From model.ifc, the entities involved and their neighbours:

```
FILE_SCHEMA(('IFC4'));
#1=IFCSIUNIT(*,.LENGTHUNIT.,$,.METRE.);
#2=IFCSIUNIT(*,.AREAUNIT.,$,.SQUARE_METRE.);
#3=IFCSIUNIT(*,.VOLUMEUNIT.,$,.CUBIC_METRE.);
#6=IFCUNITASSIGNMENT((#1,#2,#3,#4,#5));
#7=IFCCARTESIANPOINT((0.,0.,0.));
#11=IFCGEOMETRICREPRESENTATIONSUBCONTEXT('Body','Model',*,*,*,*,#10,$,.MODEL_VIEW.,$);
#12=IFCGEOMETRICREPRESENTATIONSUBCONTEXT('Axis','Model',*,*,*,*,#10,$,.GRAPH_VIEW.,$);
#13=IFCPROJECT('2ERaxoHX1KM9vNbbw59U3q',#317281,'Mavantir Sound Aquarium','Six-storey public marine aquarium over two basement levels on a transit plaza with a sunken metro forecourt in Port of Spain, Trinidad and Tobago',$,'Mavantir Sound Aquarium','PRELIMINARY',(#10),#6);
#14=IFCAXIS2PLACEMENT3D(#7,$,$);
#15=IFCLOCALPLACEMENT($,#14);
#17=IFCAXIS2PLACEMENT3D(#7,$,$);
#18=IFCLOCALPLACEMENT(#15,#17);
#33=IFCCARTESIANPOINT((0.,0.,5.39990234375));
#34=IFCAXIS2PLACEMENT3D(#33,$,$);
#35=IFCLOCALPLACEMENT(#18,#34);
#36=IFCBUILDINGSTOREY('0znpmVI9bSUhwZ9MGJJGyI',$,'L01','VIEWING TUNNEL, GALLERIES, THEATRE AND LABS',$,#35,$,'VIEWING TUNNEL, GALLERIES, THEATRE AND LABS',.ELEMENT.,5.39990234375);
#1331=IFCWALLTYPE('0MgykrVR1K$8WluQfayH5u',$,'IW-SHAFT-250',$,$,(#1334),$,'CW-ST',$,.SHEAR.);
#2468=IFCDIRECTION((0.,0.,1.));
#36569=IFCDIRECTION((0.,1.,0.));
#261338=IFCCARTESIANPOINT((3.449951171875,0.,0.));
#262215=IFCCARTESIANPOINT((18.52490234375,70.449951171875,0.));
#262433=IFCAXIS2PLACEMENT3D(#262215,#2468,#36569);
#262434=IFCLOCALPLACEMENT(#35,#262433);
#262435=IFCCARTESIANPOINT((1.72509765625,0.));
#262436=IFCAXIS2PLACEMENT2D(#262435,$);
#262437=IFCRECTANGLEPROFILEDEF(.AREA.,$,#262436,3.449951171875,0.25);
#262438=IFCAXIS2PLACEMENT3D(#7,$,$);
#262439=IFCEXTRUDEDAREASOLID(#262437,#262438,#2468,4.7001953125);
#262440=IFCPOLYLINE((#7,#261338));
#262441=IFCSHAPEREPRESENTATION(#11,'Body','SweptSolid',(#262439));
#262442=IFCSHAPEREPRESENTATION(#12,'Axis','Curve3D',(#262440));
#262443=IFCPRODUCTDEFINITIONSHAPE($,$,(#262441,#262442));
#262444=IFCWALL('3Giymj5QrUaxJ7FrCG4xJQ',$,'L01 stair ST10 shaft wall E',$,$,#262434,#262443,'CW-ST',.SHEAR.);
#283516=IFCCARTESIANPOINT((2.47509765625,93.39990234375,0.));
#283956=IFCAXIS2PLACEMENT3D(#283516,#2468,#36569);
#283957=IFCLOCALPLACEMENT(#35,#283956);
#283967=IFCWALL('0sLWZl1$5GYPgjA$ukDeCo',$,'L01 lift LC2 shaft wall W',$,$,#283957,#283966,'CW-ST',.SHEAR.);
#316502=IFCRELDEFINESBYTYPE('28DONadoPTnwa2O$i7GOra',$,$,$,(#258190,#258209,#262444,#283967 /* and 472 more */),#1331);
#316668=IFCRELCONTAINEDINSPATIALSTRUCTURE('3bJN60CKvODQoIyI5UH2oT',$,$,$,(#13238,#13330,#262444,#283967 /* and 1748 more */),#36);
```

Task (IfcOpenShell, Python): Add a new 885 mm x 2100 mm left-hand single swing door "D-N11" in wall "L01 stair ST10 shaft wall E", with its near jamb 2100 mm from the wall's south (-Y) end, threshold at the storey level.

```python
import numpy as np
import ifcopenshell
import ifcopenshell.api.feature
import ifcopenshell.api.geometry
import ifcopenshell.api.root
import ifcopenshell.api.spatial
import ifcopenshell.geom
import ifcopenshell.util.element
import ifcopenshell.util.placement
import ifcopenshell.util.representation
import ifcopenshell.util.shape
import ifcopenshell.util.unit

model = ifcopenshell.open("model.ifc")
unit_scale = ifcopenshell.util.unit.calculate_unit_scale(model)
settings = ifcopenshell.geom.settings()


def volume(element):
    """Net volume in cubic metres, openings subtracted."""
    shape = ifcopenshell.geom.create_shape(settings, element)
    return ifcopenshell.util.shape.get_volume(shape.geometry)


wall = model.by_guid("3Giymj5QrUaxJ7FrCG4xJQ")
storey = ifcopenshell.util.element.get_container(wall, ifc_class="IfcBuildingStorey")
context = ifcopenshell.util.representation.get_context(model, "Model", "Body", "MODEL_VIEW")
before = volume(wall)

width, height, from_end, sill = 0.885, 2.1, 2.1, 0.0  # metres

# The wall runs along its own X axis, and the end named is its -X end.
wall_shape = ifcopenshell.geom.create_shape(settings, wall)
x, y, z = ifcopenshell.util.shape.get_vertices(wall_shape.geometry).T
start = x.min() + from_end
face, thickness = float(y.min()), float(y.max() - y.min())
wall_matrix = ifcopenshell.util.placement.get_local_placement(wall.ObjectPlacement)
level = ifcopenshell.util.placement.get_local_placement(storey.ObjectPlacement)[2, 3]


def in_wall(x, y):
    """Placement at x, y metres in the wall's axes, at sill height."""
    matrix = wall_matrix.copy()
    matrix[:, 3] = wall_matrix @ np.array([x / unit_scale, y / unit_scale, 0.0, 1.0])
    matrix[2, 3] = level + sill / unit_scale
    return matrix


# Opening: a box that overshoots both wall faces by 50 mm.
opening = ifcopenshell.api.root.create_entity(model, ifc_class="IfcOpeningElement", predefined_type="OPENING")
box = ifcopenshell.api.geometry.add_wall_representation(
    model, context=context, length=width, height=height, thickness=thickness + 0.1
)
ifcopenshell.api.geometry.assign_representation(model, product=opening, representation=box)
ifcopenshell.api.geometry.edit_object_placement(model, product=opening, matrix=in_wall(start, face - 0.05), is_si=False)
ifcopenshell.api.feature.add_feature(model, feature=opening, element=wall)

door = ifcopenshell.api.root.create_entity(model, ifc_class="IfcDoor", name="D-N11", predefined_type="DOOR")
door.OverallWidth, door.OverallHeight = width / unit_scale, height / unit_scale
door.OperationType = "SINGLE_SWING_LEFT"
body = ifcopenshell.api.geometry.add_door_representation(
    model,
    context=context,
    overall_width=door.OverallWidth,
    overall_height=door.OverallHeight,
    operation_type="SINGLE_SWING_LEFT",
    lining_properties={"LiningDepth": thickness / unit_scale, "ThresholdDepth": thickness / unit_scale},
)
ifcopenshell.api.geometry.assign_representation(model, product=door, representation=body)
ifcopenshell.api.spatial.assign_container(model, products=[door], relating_structure=storey)
ifcopenshell.api.feature.add_filling(model, opening=opening, element=door)

# The lining spans the wall, so the door starts at the wall face.
ifcopenshell.api.geometry.edit_object_placement(model, product=door, matrix=in_wall(start, face), is_si=False)

after = volume(wall)

print(f"wall volume {before:.3f} -> {after:.3f} m3")

model.write("model_edited.ifc")
```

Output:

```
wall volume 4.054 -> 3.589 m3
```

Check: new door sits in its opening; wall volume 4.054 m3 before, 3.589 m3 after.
